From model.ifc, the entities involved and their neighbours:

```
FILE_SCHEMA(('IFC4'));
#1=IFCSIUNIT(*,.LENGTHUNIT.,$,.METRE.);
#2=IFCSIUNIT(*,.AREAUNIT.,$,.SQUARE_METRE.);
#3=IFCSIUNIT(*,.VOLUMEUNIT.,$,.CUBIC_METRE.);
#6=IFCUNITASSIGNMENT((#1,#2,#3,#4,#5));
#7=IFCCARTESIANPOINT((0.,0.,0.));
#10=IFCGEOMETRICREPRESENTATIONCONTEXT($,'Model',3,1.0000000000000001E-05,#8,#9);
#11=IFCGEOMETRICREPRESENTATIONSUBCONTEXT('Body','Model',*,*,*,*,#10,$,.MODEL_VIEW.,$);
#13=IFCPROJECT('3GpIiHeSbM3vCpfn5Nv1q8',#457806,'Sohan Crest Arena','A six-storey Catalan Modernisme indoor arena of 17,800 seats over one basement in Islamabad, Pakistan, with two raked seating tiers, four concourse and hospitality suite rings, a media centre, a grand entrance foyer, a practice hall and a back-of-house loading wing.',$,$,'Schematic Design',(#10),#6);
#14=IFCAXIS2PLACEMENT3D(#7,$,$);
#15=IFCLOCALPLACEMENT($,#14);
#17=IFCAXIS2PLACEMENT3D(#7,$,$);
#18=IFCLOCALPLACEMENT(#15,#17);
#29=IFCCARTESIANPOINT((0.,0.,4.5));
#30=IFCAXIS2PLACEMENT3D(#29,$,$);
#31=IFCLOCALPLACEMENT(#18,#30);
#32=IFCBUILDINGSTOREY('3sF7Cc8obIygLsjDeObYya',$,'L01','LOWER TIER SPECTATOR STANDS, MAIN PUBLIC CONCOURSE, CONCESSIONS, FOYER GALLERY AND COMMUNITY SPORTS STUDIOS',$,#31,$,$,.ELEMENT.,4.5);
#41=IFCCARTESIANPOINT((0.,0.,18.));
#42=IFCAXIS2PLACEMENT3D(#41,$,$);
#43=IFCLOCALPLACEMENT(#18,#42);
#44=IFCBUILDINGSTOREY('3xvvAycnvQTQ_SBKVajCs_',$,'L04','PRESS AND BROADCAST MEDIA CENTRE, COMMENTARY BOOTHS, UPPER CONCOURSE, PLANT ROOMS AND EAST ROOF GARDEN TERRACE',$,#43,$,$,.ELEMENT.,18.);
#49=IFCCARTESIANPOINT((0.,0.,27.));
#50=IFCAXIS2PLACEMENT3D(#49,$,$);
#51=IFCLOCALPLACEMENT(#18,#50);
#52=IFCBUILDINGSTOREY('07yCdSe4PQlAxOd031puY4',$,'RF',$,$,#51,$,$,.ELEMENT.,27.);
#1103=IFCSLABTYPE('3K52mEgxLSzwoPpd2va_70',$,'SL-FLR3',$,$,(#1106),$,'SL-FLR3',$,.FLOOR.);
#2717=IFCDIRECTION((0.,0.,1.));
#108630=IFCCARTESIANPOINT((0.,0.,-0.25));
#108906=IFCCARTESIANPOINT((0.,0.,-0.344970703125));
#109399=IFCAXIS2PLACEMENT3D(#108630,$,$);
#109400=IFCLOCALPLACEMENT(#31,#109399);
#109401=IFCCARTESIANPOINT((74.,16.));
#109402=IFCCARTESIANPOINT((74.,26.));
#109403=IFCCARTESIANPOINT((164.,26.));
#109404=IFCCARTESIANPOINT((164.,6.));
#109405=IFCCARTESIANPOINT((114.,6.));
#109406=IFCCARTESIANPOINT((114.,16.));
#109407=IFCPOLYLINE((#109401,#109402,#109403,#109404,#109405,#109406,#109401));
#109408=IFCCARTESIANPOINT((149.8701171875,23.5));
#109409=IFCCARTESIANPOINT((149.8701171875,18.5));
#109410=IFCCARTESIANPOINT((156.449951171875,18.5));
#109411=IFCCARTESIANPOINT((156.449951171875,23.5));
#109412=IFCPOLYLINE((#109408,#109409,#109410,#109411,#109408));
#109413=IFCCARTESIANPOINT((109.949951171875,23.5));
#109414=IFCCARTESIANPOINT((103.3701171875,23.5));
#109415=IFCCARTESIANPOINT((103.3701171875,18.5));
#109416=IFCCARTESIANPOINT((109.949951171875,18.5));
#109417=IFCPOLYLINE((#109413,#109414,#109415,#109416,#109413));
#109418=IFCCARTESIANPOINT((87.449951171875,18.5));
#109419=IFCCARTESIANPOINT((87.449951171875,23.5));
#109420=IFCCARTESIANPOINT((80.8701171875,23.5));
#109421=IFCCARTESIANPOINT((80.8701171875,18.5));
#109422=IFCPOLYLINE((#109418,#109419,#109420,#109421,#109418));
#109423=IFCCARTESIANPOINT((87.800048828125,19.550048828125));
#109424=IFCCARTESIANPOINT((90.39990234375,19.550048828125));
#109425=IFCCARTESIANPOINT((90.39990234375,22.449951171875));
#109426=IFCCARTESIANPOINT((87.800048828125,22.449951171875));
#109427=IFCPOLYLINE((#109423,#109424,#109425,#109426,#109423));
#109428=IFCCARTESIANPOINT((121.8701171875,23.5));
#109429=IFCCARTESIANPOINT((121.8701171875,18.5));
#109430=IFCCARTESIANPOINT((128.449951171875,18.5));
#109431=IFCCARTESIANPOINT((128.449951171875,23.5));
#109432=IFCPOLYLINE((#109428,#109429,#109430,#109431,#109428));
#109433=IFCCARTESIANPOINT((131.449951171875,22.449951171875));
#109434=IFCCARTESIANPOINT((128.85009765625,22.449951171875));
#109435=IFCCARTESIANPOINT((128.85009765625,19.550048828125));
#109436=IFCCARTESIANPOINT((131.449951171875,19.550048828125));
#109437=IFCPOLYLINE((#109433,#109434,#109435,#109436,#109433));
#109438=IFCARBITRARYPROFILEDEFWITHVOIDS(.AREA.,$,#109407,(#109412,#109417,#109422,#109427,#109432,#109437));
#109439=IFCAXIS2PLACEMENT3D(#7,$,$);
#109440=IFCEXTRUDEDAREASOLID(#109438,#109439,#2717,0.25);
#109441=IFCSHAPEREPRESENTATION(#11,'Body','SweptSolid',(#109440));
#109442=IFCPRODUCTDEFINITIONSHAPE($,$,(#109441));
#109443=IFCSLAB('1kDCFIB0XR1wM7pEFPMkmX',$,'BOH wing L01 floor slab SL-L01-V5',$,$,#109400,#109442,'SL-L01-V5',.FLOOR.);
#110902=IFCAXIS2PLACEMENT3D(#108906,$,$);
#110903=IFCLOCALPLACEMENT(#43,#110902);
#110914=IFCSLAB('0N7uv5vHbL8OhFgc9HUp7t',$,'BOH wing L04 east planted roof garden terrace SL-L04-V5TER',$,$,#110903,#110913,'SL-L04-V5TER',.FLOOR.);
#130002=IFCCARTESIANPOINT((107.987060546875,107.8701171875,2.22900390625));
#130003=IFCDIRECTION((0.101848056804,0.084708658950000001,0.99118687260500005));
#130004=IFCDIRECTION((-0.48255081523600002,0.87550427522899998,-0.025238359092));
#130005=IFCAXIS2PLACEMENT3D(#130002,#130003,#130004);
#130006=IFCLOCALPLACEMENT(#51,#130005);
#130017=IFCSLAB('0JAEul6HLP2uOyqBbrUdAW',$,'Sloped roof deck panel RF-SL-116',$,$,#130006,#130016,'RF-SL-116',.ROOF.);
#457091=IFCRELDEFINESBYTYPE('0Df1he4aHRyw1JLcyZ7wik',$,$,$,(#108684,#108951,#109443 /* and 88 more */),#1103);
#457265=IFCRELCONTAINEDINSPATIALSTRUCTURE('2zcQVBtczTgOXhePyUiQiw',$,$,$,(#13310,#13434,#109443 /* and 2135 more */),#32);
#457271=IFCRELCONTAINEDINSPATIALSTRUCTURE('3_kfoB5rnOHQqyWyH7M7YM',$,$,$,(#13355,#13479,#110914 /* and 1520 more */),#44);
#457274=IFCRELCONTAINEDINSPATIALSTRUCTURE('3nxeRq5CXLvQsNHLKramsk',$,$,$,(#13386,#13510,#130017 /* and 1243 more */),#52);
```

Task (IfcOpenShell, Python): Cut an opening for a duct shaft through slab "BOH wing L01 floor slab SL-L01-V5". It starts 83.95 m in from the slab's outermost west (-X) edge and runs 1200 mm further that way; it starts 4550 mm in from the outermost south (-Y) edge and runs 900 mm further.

```python
import numpy as np
import ifcopenshell
import ifcopenshell.api.feature
import ifcopenshell.api.geometry
import ifcopenshell.api.root
import ifcopenshell.geom
import ifcopenshell.util.placement
import ifcopenshell.util.representation
import ifcopenshell.util.shape
import ifcopenshell.util.unit

model = ifcopenshell.open("model.ifc")
unit_scale = ifcopenshell.util.unit.calculate_unit_scale(model)
settings = ifcopenshell.geom.settings()


def volume(element):
    """Net volume in cubic metres, openings subtracted."""
    shape = ifcopenshell.geom.create_shape(settings, element)
    return ifcopenshell.util.shape.get_volume(shape.geometry)


slab = model.by_guid("1kDCFIB0XR1wM7pEFPMkmX")
before = volume(slab)

# Extent in the slab's own axes, in metres. The edges named are its -X and -Y sides.
slab_shape = ifcopenshell.geom.create_shape(settings, slab)
vertices = ifcopenshell.util.shape.get_vertices(slab_shape.geometry)
x_min, y_min, bottom = vertices.min(axis=0)
top = vertices[:, 2].max()

opening = ifcopenshell.api.root.create_entity(model, ifc_class="IfcOpeningElement", name="Duct shaft opening", predefined_type="OPENING")
context = ifcopenshell.util.representation.get_context(model, "Model", "Body", "MODEL_VIEW")
width, depth = 1.2, 0.9
outline = [(0.0, 0.0), (width, 0.0), (width, depth), (0.0, depth), (0.0, 0.0)]
# Overshoot both faces by 50 mm so the cut is clean.
shape = ifcopenshell.api.geometry.add_slab_representation(
    model, context=context, depth=top - bottom + 0.1, polyline=outline
)
ifcopenshell.api.geometry.assign_representation(model, product=opening, representation=shape)

matrix = ifcopenshell.util.placement.get_local_placement(slab.ObjectPlacement)
matrix[:, 3] = matrix @ np.append(np.array([x_min + 83.95, y_min + 4.55, bottom - 0.05]) / unit_scale, 1.0)
ifcopenshell.api.geometry.edit_object_placement(model, product=opening, matrix=matrix, is_si=False)
ifcopenshell.api.feature.add_feature(model, feature=opening, element=slab)

after = volume(slab)

print(f"slab volume {before:.3f} -> {after:.3f} m3")

model.write("model_edited.ifc")
```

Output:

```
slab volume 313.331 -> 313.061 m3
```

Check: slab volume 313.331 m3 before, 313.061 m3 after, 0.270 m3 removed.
